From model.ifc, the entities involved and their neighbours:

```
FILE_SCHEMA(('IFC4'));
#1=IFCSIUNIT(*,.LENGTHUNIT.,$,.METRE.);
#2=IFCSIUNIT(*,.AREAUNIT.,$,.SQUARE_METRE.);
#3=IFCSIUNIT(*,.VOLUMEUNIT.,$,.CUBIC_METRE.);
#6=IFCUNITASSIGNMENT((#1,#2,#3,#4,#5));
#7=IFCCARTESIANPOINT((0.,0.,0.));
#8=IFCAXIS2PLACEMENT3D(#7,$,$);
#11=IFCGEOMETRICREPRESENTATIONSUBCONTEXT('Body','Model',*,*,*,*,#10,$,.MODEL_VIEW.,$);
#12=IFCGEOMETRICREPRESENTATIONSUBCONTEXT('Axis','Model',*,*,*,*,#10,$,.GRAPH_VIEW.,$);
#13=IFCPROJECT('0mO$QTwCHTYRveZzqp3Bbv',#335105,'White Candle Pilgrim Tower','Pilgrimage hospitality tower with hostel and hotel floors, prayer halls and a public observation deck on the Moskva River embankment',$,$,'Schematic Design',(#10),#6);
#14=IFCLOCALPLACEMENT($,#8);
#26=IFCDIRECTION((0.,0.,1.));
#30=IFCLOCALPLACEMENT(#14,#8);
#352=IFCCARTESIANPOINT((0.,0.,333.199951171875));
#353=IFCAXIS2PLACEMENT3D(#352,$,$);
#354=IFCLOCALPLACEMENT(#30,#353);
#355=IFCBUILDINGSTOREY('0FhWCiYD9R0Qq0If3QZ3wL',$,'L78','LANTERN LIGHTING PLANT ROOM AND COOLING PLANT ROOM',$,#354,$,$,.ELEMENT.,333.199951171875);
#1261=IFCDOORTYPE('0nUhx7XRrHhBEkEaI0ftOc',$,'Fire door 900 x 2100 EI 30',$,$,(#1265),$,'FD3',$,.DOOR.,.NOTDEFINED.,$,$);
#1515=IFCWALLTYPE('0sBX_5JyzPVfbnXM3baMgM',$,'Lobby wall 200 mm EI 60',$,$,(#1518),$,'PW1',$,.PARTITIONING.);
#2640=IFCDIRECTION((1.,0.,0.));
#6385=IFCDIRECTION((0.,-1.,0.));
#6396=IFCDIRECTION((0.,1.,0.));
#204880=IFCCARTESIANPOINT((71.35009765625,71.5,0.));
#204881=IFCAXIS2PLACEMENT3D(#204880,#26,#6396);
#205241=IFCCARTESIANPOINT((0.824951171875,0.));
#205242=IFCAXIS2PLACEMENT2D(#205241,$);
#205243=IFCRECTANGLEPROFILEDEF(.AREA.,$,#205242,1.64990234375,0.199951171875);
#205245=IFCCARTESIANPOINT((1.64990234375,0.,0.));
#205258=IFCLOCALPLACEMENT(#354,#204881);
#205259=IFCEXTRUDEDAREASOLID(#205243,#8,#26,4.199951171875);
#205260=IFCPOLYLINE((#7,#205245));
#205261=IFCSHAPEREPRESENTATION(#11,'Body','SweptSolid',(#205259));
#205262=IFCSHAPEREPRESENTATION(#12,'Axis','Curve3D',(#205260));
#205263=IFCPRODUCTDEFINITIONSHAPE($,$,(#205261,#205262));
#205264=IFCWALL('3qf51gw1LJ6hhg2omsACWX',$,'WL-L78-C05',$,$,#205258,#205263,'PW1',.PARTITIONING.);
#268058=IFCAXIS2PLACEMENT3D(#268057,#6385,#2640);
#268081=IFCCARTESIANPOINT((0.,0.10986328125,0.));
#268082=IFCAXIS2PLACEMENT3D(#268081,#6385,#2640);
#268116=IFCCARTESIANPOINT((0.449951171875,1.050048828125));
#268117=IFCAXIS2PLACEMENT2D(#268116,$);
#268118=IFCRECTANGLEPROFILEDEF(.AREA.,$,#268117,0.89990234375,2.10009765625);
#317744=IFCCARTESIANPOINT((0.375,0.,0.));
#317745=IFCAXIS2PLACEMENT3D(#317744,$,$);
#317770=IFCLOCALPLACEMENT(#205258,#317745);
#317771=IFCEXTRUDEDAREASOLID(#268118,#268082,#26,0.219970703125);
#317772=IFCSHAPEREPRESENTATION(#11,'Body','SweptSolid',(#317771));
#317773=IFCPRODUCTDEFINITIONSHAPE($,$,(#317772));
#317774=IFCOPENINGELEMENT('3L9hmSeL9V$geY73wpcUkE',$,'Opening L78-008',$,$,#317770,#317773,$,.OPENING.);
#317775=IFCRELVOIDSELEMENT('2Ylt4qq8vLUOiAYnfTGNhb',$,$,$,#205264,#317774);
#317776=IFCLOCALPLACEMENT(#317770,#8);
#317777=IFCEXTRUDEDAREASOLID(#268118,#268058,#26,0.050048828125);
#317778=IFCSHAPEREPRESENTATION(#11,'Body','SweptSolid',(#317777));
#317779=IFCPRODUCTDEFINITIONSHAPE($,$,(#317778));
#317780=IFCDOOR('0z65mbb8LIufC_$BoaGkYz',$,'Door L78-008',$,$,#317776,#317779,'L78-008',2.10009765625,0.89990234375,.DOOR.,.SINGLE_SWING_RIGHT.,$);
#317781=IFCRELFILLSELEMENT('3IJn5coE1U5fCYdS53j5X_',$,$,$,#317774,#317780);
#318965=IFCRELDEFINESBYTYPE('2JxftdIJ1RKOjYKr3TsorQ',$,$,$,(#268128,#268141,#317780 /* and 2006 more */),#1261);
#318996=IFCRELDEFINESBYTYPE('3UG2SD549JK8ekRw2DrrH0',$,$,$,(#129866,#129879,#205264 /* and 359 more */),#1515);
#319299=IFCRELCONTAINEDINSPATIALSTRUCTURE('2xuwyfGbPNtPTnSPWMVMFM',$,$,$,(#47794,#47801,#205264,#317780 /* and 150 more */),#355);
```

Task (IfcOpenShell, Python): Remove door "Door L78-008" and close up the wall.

```python
import ifcopenshell
import ifcopenshell.api.feature
import ifcopenshell.api.root
import ifcopenshell.geom
import ifcopenshell.util.shape

model = ifcopenshell.open("model.ifc")
settings = ifcopenshell.geom.settings()


def volume(element):
    """Net volume in cubic metres, openings subtracted."""
    shape = ifcopenshell.geom.create_shape(settings, element)
    return ifcopenshell.util.shape.get_volume(shape.geometry)


door = model.by_guid("0z65mbb8LIufC_$BoaGkYz")
opening = door.FillsVoids[0].RelatingOpeningElement
wall = opening.VoidsElements[0].RelatingBuildingElement
before = volume(wall)

ifcopenshell.api.root.remove_product(model, product=door)
ifcopenshell.api.feature.remove_feature(model, feature=opening)

after = volume(wall)

print(f"wall volume {before:.3f} -> {after:.3f} m3")

model.write("model_edited.ifc")
```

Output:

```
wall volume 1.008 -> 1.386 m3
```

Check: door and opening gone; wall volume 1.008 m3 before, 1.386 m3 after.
